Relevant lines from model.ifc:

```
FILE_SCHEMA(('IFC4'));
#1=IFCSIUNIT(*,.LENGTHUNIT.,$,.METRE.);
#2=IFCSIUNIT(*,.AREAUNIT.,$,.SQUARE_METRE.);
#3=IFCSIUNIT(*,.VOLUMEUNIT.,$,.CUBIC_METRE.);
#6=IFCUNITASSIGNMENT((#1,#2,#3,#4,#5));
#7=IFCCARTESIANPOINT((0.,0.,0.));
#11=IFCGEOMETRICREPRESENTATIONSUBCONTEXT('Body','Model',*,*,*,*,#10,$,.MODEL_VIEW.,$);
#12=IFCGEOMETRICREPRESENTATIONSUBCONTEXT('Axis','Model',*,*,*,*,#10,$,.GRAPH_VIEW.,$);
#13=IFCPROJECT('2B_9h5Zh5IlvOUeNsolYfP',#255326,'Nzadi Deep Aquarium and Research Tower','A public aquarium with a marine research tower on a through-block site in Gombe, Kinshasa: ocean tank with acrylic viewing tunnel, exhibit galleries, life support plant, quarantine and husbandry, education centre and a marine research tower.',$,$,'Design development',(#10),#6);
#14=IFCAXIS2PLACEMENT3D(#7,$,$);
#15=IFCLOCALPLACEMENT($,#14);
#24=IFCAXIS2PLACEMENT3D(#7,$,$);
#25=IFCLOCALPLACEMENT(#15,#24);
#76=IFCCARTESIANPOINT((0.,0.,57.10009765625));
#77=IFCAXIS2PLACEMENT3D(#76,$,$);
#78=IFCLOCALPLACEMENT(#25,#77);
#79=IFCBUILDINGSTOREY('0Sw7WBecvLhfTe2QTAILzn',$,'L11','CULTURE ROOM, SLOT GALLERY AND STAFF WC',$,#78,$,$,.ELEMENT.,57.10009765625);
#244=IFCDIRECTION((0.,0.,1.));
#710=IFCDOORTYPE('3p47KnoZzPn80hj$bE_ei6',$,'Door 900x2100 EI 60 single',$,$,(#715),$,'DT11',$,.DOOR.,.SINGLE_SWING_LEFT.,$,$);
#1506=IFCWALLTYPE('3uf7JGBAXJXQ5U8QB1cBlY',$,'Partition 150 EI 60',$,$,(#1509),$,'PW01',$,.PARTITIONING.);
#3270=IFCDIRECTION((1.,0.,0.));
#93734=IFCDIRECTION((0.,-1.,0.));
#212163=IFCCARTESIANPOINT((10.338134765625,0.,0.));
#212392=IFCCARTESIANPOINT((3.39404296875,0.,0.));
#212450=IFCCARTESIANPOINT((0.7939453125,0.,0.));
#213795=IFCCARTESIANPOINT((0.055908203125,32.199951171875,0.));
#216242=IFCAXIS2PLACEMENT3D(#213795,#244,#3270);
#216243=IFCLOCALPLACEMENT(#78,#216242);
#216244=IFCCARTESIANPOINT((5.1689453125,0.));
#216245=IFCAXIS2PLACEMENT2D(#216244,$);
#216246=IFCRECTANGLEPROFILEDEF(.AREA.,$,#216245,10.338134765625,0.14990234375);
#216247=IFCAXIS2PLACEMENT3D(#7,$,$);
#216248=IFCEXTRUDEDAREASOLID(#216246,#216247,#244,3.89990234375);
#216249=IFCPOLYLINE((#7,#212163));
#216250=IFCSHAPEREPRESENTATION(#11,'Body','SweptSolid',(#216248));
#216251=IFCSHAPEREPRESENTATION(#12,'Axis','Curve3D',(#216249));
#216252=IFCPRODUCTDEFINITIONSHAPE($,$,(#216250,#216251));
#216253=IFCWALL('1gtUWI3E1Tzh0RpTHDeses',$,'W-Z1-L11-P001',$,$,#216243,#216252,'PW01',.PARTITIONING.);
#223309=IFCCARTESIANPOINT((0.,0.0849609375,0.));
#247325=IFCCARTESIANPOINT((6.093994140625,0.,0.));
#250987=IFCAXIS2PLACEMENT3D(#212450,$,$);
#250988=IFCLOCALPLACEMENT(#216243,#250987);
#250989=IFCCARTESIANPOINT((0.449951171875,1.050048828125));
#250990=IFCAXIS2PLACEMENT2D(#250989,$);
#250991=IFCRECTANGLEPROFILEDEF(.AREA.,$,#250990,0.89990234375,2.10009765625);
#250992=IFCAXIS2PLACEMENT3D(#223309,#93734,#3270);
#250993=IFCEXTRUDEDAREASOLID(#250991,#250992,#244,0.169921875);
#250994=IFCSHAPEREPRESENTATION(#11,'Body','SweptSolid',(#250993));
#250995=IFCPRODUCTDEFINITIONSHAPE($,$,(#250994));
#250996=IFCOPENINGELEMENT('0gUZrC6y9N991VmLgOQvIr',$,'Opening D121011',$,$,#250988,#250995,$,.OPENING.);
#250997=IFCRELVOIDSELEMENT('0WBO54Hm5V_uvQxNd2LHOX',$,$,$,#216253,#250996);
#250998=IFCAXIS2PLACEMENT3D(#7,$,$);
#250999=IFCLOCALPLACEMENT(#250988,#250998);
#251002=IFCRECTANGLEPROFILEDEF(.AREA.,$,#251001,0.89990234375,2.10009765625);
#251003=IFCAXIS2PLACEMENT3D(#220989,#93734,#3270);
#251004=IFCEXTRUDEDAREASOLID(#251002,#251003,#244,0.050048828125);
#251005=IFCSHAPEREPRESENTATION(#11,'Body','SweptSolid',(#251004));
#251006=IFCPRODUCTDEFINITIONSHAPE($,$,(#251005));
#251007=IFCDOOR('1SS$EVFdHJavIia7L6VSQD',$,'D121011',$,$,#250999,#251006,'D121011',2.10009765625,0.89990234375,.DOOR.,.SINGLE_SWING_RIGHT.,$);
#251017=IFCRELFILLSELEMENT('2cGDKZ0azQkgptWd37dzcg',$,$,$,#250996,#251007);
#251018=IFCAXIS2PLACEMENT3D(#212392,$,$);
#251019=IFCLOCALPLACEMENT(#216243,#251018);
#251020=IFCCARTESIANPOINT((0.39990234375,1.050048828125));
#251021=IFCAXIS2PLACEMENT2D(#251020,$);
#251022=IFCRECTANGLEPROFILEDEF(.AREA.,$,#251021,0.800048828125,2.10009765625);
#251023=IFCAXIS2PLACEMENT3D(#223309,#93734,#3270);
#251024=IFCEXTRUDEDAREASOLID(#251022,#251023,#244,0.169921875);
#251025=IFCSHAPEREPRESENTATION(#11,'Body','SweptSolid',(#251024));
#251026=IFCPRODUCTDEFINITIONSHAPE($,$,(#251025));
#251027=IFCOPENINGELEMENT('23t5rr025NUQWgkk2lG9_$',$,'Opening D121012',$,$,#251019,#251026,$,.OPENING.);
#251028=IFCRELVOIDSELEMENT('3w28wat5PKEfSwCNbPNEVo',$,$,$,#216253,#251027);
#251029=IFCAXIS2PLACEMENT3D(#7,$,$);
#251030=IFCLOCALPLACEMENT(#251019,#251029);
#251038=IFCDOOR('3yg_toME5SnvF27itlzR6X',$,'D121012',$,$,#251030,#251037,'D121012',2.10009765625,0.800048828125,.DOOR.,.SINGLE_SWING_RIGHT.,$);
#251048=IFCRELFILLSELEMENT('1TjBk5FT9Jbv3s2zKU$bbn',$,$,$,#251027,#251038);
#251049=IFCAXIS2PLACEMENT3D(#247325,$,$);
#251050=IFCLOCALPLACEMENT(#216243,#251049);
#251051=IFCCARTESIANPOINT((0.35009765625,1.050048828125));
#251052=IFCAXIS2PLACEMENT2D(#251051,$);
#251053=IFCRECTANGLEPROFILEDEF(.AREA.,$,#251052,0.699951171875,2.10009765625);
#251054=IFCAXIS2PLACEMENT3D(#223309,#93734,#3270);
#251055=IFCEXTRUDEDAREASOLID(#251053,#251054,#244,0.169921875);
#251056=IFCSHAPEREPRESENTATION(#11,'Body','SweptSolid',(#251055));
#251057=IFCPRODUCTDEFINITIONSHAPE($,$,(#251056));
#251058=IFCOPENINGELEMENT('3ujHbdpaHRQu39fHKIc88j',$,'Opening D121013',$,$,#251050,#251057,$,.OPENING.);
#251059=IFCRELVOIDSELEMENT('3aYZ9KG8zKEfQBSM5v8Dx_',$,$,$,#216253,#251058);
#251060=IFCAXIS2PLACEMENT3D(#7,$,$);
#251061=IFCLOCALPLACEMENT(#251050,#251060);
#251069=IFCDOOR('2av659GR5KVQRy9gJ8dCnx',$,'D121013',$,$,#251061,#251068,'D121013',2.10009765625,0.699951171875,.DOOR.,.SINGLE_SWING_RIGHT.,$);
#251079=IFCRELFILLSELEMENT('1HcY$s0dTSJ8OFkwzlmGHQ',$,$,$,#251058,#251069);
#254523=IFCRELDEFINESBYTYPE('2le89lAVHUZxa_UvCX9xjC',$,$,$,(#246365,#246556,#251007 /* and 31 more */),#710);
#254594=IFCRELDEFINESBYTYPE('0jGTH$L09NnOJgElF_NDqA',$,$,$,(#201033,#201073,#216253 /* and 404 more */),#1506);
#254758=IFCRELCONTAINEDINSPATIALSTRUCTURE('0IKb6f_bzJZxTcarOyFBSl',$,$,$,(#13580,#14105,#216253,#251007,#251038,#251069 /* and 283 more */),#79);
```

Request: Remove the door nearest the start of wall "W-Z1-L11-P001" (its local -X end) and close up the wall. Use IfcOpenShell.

```python
import ifcopenshell
import ifcopenshell.api.feature
import ifcopenshell.api.root
import ifcopenshell.geom
import ifcopenshell.util.shape

model = ifcopenshell.open("model.ifc")
settings = ifcopenshell.geom.settings()


def volume(element):
    """Net volume in cubic metres, openings subtracted."""
    shape = ifcopenshell.geom.create_shape(settings, element)
    return ifcopenshell.util.shape.get_volume(shape.geometry)


door = model.by_id(251007)
opening = door.FillsVoids[0].RelatingOpeningElement
wall = opening.VoidsElements[0].RelatingBuildingElement
before = volume(wall)

ifcopenshell.api.root.remove_product(model, product=door)
ifcopenshell.api.feature.remove_feature(model, feature=opening)

after = volume(wall)

print(f"wall volume {before:.3f} -> {after:.3f} m3")

model.write("model_rev.ifc")
```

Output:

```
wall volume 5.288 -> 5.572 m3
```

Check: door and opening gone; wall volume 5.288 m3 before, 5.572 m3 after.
